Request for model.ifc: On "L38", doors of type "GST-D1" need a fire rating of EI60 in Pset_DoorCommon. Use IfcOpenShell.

First a look at what the model holds.

```python
import ifcopenshell
import ifcopenshell.util.element

model = ifcopenshell.open("model.ifc")
print(model.schema)
storey = next(s for s in model.by_type("IfcBuildingStorey") if s.Name == "L38")
doors = [e for e in ifcopenshell.util.element.get_decomposition(storey) if e.is_a("IfcDoor")]
seen = {}
for e in doors:
    element_type = ifcopenshell.util.element.get_type(e)
    key = (element_type.Name if element_type != e and element_type else None, ifcopenshell.util.element.get_pset(e, "Pset_DoorCommon", "FireRating"))
    seen[key] = seen.get(key, 0) + 1
for (name, value), count in sorted(seen.items(), key=str):
    print(count, "x", name, "|", value)
```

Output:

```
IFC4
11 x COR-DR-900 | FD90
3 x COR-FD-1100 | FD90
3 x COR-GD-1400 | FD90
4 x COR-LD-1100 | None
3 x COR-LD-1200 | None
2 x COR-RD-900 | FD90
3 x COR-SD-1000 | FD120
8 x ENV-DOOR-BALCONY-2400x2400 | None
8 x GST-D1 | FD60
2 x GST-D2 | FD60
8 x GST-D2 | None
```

```python
import ifcopenshell
import ifcopenshell.api.pset
import ifcopenshell.util.element

model = ifcopenshell.open("model.ifc")

storey = next(s for s in model.by_type("IfcBuildingStorey") if s.Name == "L38")
doors = [e for e in ifcopenshell.util.element.get_decomposition(storey) if e.is_a("IfcDoor")]

count = 0
for e in doors:
    element_type = ifcopenshell.util.element.get_type(e)
    if element_type in (None, e) or element_type.Name != "GST-D1":
        continue
    found = ifcopenshell.util.element.get_pset(e, "Pset_DoorCommon", should_inherit=False)
    if found:
        pset = model.by_id(found["id"])
        if len(ifcopenshell.util.element.get_elements_by_pset(pset)) > 1:
            pset = ifcopenshell.api.pset.unshare_pset(model, products=[e], pset=pset)[0]
    else:
        pset = ifcopenshell.api.pset.add_pset(model, product=e, name="Pset_DoorCommon")
    ifcopenshell.api.pset.edit_pset(model, pset=pset, properties={"FireRating": "EI60"})
    count += 1

print(count, "doors updated")

model.write("model_edited.ifc")
```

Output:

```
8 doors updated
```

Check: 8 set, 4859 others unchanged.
